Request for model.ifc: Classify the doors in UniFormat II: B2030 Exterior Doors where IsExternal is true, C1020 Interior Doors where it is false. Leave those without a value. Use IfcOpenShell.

First a look at what the model holds.

```python
import ifcopenshell
import ifcopenshell.util.element

model = ifcopenshell.open("model.ifc")
print(model.schema)
print("classifications:", [c.Name for c in model.by_type("IfcClassification")])
values = [ifcopenshell.util.element.get_pset(e, "Pset_DoorCommon", "IsExternal") for e in model.by_type("IfcDoor")]
for value in (True, False, None):
    print("IsExternal", value, values.count(value))
```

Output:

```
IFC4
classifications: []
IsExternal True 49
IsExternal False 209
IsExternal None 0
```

```python
import ifcopenshell
import ifcopenshell.api.classification
import ifcopenshell.util.element

model = ifcopenshell.open("model.ifc")

system = ifcopenshell.api.classification.add_classification(model, classification="UniFormat II")

doors = model.by_type("IfcDoor")
external = {e: ifcopenshell.util.element.get_pset(e, "Pset_DoorCommon", "IsExternal") for e in doors}
for flag, code, name in ((True, "B2030", "Exterior Doors"), (False, "C1020", "Interior Doors")):
    products = [e for e in doors if external[e] is flag]
    ifcopenshell.api.classification.add_reference(
        model, products=products, classification=system, identification=code, name=name
    )
    print(code, len(products))

model.write("model_edited.ifc")
```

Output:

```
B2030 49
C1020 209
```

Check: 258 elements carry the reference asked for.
